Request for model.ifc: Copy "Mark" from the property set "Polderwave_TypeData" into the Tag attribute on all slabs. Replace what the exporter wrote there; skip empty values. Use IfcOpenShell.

First a look at what the model holds.

```python
import ifcopenshell
import ifcopenshell.util.element

model = ifcopenshell.open("model.ifc")
print(model.schema)
slabs = model.by_type("IfcSlab")
print(len(slabs), "slabs")
for e in slabs[:8]:
    source = ifcopenshell.util.element.get_pset(e, "Polderwave_TypeData", "Mark")
    target = e.Tag
    print(e.id(), repr(source), repr(target), sep=" | ")
```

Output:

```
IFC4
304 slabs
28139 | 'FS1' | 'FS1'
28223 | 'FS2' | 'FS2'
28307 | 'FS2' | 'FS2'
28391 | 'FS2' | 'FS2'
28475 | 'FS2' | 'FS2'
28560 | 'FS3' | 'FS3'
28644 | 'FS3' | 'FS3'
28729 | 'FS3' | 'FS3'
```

```python
import ifcopenshell
import ifcopenshell.util.element

model = ifcopenshell.open("model.ifc")

count = 0
for e in model.by_type("IfcSlab"):
    value = ifcopenshell.util.element.get_pset(e, "Polderwave_TypeData", "Mark")
    current = e.Tag
    if not value or not value.strip() or current == value:
        continue
    e.Tag = value
    count += 1

print(count, "slabs updated")

model.write("model_v2.ifc")
```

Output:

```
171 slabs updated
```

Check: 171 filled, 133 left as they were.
